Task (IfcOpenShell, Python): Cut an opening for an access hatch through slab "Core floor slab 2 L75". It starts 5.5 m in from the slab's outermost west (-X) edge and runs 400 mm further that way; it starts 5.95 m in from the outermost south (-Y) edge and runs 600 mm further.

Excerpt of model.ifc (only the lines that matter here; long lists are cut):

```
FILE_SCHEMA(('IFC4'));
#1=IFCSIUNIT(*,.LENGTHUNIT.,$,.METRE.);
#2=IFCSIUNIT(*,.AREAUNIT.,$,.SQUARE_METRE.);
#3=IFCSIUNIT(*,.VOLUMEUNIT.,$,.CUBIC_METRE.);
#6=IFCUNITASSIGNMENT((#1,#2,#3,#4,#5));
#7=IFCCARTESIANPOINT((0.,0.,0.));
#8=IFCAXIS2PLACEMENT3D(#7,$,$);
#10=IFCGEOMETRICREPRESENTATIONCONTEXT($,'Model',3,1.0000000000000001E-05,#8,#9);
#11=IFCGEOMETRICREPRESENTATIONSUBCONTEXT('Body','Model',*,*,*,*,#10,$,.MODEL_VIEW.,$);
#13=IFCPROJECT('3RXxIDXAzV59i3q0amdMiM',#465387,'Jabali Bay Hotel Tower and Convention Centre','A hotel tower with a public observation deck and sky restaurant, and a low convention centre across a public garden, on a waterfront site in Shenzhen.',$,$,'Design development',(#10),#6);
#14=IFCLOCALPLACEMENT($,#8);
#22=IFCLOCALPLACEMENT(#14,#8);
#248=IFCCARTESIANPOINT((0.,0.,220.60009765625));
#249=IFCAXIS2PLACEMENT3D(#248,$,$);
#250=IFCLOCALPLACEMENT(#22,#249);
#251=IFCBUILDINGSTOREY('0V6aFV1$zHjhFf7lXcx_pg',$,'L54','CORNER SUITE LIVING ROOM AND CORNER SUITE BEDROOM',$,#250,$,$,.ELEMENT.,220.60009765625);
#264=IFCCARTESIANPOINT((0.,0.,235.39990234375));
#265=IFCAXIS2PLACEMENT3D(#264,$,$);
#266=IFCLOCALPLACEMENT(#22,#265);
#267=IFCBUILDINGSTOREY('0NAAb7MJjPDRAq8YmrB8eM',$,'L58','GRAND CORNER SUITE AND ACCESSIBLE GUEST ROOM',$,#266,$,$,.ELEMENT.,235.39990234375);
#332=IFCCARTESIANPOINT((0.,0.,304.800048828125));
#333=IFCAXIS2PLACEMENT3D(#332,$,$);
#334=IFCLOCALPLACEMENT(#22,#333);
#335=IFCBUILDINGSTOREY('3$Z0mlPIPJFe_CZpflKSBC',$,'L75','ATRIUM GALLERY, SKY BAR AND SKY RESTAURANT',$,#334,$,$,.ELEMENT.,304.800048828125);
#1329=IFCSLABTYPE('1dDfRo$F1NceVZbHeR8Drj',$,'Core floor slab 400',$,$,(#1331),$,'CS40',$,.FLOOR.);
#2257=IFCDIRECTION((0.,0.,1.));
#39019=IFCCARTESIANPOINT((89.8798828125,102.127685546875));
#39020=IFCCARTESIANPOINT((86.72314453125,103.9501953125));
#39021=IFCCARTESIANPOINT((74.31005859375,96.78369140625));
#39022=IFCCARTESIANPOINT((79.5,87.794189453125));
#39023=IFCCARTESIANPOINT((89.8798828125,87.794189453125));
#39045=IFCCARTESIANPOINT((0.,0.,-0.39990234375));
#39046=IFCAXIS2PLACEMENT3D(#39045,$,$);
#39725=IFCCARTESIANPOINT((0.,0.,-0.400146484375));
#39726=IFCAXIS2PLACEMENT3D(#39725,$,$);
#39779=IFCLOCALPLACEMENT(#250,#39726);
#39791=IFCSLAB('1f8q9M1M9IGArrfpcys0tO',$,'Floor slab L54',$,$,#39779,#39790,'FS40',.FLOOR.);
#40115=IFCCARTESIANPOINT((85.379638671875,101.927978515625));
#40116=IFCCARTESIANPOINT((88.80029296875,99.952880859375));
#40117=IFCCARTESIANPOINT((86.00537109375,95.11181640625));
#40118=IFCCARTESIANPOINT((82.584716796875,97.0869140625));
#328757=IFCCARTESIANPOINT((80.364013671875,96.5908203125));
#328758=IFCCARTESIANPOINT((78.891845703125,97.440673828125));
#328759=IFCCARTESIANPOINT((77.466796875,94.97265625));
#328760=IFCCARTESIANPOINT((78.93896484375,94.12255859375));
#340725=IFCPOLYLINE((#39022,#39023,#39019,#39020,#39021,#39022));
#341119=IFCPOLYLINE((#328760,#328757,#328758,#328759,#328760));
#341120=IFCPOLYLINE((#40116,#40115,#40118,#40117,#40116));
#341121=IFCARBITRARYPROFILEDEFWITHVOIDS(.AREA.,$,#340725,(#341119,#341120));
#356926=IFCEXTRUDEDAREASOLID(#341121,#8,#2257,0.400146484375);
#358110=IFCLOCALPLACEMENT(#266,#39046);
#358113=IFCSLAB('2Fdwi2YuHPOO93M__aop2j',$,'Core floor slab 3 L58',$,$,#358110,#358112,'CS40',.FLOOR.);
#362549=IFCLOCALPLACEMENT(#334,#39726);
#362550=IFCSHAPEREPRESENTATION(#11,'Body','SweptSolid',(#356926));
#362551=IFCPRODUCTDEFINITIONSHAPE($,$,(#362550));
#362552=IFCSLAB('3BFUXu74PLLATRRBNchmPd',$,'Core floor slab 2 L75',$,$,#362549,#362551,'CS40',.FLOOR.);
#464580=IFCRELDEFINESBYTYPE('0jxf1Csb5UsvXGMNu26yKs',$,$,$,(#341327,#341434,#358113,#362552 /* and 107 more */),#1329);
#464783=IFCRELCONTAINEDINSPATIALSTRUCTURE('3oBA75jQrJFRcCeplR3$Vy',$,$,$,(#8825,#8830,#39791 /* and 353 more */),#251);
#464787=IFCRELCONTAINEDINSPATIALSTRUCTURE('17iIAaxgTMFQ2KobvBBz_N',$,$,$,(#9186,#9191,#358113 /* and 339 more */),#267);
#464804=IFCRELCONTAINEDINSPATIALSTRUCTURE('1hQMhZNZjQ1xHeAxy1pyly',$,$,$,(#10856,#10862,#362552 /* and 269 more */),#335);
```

```python
import numpy as np
import ifcopenshell
import ifcopenshell.api.feature
import ifcopenshell.api.geometry
import ifcopenshell.api.root
import ifcopenshell.geom
import ifcopenshell.util.placement
import ifcopenshell.util.representation
import ifcopenshell.util.shape
import ifcopenshell.util.unit

model = ifcopenshell.open("model.ifc")
unit_scale = ifcopenshell.util.unit.calculate_unit_scale(model)
settings = ifcopenshell.geom.settings()


def volume(element):
    """Net volume in cubic metres, openings subtracted."""
    shape = ifcopenshell.geom.create_shape(settings, element)
    return ifcopenshell.util.shape.get_volume(shape.geometry)


slab = model.by_guid("3BFUXu74PLLATRRBNchmPd")
before = volume(slab)

# Extent in the slab's own axes, in metres. The edges named are its -X and -Y sides.
slab_shape = ifcopenshell.geom.create_shape(settings, slab)
vertices = ifcopenshell.util.shape.get_vertices(slab_shape.geometry)
x_min, y_min, bottom = vertices.min(axis=0)
top = vertices[:, 2].max()

opening = ifcopenshell.api.root.create_entity(model, ifc_class="IfcOpeningElement", name="Access hatch opening", predefined_type="OPENING")
context = ifcopenshell.util.representation.get_context(model, "Model", "Body", "MODEL_VIEW")
width, depth = 0.4, 0.6
outline = [(0.0, 0.0), (width, 0.0), (width, depth), (0.0, depth), (0.0, 0.0)]
# Overshoot both faces by 50 mm so the cut is clean.
shape = ifcopenshell.api.geometry.add_slab_representation(
    model, context=context, depth=top - bottom + 0.1, polyline=outline
)
ifcopenshell.api.geometry.assign_representation(model, product=opening, representation=shape)

matrix = ifcopenshell.util.placement.get_local_placement(slab.ObjectPlacement)
matrix[:, 3] = matrix @ np.append(np.array([x_min + 5.5, y_min + 5.95, bottom - 0.05]) / unit_scale, 1.0)
ifcopenshell.api.geometry.edit_object_placement(model, product=opening, matrix=matrix, is_si=False)
ifcopenshell.api.feature.add_feature(model, feature=opening, element=slab)

after = volume(slab)

print(f"slab volume {before:.3f} -> {after:.3f} m3")

model.write("model_v2.ifc")
```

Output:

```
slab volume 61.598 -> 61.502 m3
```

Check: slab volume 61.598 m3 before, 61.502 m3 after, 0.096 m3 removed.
